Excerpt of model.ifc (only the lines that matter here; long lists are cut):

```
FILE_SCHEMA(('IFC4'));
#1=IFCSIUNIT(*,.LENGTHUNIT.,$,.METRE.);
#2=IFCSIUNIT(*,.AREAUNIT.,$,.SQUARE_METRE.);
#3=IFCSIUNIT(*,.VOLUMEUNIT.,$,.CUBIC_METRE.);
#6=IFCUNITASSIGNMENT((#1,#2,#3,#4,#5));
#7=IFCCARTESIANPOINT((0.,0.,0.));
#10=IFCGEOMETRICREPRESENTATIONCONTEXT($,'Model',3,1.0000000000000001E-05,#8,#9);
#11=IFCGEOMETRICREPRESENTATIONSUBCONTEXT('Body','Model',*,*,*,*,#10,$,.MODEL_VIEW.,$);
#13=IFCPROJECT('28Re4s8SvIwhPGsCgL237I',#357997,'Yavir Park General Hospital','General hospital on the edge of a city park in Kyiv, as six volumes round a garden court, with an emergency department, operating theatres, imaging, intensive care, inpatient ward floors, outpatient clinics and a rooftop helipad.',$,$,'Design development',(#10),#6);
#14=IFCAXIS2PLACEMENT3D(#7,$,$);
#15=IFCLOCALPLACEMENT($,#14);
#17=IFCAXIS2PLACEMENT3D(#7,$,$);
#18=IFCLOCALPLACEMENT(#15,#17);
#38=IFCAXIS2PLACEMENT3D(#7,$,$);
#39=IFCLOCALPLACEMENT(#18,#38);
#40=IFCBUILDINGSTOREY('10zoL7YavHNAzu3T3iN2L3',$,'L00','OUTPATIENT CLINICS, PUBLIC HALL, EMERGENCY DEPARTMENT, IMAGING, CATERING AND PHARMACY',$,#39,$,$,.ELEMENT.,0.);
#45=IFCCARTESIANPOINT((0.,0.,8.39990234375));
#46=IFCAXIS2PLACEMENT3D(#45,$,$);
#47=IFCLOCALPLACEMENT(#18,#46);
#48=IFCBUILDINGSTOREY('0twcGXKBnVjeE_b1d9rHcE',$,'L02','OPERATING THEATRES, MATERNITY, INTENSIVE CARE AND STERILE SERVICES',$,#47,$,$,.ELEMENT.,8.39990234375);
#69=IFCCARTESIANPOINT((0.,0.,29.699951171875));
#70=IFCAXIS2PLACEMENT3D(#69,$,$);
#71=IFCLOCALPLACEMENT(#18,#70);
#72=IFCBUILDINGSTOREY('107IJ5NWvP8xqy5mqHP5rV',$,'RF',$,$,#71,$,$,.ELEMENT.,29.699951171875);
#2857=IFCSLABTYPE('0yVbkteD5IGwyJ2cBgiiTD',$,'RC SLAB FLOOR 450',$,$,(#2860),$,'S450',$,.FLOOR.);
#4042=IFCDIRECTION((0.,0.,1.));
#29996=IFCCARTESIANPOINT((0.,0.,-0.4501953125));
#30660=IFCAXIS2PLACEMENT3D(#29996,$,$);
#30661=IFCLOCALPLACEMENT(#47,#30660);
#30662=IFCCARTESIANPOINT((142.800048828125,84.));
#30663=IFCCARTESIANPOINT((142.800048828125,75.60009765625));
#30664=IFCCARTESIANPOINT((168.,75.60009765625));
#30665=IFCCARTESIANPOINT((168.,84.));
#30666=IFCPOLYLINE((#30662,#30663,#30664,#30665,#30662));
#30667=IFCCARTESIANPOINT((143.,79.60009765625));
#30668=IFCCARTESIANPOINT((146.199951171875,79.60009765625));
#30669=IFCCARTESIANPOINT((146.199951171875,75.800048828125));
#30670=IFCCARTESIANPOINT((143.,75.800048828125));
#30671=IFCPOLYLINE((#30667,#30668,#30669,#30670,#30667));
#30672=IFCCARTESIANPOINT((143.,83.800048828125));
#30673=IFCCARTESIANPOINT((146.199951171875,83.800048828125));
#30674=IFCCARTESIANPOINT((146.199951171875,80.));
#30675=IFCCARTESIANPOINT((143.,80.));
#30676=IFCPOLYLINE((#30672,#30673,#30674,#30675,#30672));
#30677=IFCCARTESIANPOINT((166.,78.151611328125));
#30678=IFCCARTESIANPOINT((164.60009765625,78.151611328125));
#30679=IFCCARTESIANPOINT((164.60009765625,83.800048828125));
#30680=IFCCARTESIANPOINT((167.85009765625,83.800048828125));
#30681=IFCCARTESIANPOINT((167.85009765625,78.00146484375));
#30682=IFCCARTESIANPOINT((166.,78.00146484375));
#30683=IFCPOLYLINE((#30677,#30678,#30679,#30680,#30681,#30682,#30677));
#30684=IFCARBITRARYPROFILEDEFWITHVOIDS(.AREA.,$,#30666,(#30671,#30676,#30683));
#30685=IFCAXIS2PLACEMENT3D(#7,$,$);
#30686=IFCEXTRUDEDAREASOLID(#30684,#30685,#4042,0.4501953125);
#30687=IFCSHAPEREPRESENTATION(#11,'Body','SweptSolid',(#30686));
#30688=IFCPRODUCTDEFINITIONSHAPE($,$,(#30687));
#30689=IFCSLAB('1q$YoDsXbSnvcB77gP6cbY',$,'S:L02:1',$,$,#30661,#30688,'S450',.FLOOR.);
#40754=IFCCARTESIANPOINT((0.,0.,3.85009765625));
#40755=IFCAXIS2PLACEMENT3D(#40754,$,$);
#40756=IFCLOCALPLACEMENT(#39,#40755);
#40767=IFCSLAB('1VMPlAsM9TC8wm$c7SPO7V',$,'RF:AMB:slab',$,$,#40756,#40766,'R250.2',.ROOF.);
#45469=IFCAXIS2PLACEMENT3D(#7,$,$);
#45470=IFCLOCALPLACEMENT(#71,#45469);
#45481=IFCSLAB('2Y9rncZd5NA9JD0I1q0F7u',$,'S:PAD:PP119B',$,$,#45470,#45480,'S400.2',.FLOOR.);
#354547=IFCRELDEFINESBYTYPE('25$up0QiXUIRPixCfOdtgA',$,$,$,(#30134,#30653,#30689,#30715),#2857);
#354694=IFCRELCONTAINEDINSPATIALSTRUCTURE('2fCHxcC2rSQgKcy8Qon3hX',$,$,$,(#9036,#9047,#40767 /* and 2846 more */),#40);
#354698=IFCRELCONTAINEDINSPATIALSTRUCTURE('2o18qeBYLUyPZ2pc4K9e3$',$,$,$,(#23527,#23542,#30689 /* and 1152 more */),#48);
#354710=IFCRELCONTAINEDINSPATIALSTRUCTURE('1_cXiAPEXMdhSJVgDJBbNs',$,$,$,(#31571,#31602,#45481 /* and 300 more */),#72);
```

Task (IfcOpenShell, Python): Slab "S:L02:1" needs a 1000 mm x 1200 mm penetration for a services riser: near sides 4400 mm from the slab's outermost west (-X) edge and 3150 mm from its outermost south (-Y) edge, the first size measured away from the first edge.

```python
import numpy as np
import ifcopenshell
import ifcopenshell.api.feature
import ifcopenshell.api.geometry
import ifcopenshell.api.root
import ifcopenshell.geom
import ifcopenshell.util.placement
import ifcopenshell.util.representation
import ifcopenshell.util.shape
import ifcopenshell.util.unit

model = ifcopenshell.open("model.ifc")
unit_scale = ifcopenshell.util.unit.calculate_unit_scale(model)
settings = ifcopenshell.geom.settings()


def volume(element):
    """Net volume in cubic metres, openings subtracted."""
    shape = ifcopenshell.geom.create_shape(settings, element)
    return ifcopenshell.util.shape.get_volume(shape.geometry)


slab = model.by_id(30689)
before = volume(slab)

# Extent in the slab's own axes, in metres. The edges named are its -X and -Y sides.
slab_shape = ifcopenshell.geom.create_shape(settings, slab)
vertices = ifcopenshell.util.shape.get_vertices(slab_shape.geometry)
x_min, y_min, bottom = vertices.min(axis=0)
top = vertices[:, 2].max()

opening = ifcopenshell.api.root.create_entity(model, ifc_class="IfcOpeningElement", name="Services riser opening", predefined_type="OPENING")
context = ifcopenshell.util.representation.get_context(model, "Model", "Body", "MODEL_VIEW")
width, depth = 1, 1.2
outline = [(0.0, 0.0), (width, 0.0), (width, depth), (0.0, depth), (0.0, 0.0)]
# Overshoot both faces by 50 mm so the cut is clean.
shape = ifcopenshell.api.geometry.add_slab_representation(
    model, context=context, depth=top - bottom + 0.1, polyline=outline
)
ifcopenshell.api.geometry.assign_representation(model, product=opening, representation=shape)

matrix = ifcopenshell.util.placement.get_local_placement(slab.ObjectPlacement)
matrix[:, 3] = matrix @ np.append(np.array([x_min + 4.4, y_min + 3.15, bottom - 0.05]) / unit_scale, 1.0)
ifcopenshell.api.geometry.edit_object_placement(model, product=opening, matrix=matrix, is_si=False)
ifcopenshell.api.feature.add_feature(model, feature=opening, element=slab)

after = volume(slab)

print(f"slab volume {before:.3f} -> {after:.3f} m3")

model.write("model_v2.ifc")
```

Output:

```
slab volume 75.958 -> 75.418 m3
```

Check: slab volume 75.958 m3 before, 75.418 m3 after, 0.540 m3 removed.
